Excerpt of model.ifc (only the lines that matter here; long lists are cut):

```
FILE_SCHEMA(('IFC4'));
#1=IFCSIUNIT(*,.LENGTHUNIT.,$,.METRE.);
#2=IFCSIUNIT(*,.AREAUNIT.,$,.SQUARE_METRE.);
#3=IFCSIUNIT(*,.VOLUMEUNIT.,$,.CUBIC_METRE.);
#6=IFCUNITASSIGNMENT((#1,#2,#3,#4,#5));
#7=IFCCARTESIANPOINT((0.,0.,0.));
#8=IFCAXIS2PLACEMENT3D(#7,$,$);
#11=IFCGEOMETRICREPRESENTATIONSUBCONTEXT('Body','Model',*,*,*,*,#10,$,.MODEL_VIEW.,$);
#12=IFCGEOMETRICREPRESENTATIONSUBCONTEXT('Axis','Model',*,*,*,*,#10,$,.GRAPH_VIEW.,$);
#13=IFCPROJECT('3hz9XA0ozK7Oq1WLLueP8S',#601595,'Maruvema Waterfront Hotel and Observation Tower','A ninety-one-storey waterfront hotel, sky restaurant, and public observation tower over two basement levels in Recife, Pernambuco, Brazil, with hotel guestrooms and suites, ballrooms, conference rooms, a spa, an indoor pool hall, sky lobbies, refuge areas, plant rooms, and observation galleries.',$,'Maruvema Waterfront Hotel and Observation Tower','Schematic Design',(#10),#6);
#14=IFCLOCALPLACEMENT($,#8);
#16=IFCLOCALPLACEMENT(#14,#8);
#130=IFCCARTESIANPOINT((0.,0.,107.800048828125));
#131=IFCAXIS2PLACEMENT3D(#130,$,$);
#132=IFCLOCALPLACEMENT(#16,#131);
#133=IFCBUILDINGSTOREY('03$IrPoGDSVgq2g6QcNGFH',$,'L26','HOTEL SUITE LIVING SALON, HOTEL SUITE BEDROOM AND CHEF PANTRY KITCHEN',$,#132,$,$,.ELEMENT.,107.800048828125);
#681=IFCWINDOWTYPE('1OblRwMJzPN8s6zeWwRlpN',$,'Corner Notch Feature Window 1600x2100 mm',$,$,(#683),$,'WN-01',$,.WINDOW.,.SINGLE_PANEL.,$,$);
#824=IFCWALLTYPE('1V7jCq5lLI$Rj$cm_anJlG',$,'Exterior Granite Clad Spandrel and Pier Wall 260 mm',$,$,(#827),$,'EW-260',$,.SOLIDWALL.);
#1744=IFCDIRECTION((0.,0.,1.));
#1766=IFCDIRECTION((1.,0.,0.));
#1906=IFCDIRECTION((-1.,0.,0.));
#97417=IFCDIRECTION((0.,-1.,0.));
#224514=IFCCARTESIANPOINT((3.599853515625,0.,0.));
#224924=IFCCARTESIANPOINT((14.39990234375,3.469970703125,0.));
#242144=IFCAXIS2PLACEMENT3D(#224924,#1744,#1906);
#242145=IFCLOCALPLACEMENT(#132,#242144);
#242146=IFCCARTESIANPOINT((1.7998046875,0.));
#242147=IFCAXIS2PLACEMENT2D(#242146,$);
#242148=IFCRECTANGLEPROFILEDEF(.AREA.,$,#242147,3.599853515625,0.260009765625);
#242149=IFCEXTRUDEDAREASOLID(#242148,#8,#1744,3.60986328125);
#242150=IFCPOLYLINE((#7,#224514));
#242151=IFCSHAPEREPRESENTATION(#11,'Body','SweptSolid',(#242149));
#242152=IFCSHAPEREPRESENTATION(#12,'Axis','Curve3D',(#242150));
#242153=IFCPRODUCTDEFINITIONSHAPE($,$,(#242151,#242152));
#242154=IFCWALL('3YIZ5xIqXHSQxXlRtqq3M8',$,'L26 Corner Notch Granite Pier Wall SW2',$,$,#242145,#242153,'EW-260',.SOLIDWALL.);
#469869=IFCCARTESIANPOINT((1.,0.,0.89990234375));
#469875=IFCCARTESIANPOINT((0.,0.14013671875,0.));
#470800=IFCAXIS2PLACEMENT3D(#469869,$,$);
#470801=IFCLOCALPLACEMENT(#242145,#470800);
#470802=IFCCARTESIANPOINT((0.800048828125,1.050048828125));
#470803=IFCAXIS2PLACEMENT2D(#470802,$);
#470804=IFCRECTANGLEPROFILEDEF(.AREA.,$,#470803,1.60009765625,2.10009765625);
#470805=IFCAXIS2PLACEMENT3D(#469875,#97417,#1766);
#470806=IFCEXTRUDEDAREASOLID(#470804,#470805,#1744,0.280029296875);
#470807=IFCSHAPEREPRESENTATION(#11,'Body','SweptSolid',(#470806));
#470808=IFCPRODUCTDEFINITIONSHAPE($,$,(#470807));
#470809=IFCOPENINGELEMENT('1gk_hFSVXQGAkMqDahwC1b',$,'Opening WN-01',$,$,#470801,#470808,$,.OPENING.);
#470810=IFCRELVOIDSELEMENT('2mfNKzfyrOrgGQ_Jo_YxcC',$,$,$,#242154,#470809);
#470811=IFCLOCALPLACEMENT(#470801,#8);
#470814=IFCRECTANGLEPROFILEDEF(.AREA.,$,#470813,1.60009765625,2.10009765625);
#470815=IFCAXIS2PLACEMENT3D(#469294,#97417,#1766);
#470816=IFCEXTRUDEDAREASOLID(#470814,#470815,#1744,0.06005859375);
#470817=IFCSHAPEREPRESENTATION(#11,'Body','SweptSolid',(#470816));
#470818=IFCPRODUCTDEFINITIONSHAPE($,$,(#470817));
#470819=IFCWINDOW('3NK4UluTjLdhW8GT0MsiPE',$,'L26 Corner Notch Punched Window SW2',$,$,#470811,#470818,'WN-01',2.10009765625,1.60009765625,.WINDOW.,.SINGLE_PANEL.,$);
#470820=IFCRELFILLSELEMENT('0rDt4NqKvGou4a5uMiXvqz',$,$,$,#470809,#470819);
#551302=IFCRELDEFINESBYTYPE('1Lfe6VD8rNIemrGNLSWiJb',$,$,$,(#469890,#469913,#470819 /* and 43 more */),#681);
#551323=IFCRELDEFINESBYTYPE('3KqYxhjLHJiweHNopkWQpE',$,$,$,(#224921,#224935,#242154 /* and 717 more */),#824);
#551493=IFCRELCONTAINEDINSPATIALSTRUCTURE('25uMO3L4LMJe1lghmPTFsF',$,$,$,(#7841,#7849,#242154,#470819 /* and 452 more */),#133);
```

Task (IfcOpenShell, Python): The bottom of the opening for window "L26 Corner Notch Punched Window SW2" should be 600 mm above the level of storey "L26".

```python
import numpy as np
import ifcopenshell
import ifcopenshell.api.geometry
import ifcopenshell.geom
import ifcopenshell.util.element
import ifcopenshell.util.placement
import ifcopenshell.util.shape
import ifcopenshell.util.unit

model = ifcopenshell.open("model.ifc")
unit_scale = ifcopenshell.util.unit.calculate_unit_scale(model)

window = model.by_guid("3NK4UluTjLdhW8GT0MsiPE")
opening = window.FillsVoids[0].RelatingOpeningElement
storey = ifcopenshell.util.element.get_container(window, ifc_class="IfcBuildingStorey")
level = ifcopenshell.util.placement.get_local_placement(storey.ObjectPlacement)[2, 3]

# The opening's origin need not be at the sill, so measure its lowest point.
shape = ifcopenshell.geom.create_shape(ifcopenshell.geom.settings(), opening)
bottom = ifcopenshell.util.shape.get_shape_bottom_elevation(shape, shape.geometry) / unit_scale
dz = level + 0.6 / unit_scale - bottom

shift = np.array([0.0, 0.0, dz])
# The window is placed relative to its opening, so it follows when the opening moves.
matrix = ifcopenshell.util.placement.get_local_placement(opening.ObjectPlacement)
matrix[:3, 3] += shift
ifcopenshell.api.geometry.edit_object_placement(
    model, product=opening, matrix=matrix, is_si=False, should_transform_children=True
)

print(f"moved by {dz * unit_scale:+.3f} m")

model.write("model_updated.ifc")
```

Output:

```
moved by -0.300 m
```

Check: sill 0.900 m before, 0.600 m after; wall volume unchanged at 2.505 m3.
